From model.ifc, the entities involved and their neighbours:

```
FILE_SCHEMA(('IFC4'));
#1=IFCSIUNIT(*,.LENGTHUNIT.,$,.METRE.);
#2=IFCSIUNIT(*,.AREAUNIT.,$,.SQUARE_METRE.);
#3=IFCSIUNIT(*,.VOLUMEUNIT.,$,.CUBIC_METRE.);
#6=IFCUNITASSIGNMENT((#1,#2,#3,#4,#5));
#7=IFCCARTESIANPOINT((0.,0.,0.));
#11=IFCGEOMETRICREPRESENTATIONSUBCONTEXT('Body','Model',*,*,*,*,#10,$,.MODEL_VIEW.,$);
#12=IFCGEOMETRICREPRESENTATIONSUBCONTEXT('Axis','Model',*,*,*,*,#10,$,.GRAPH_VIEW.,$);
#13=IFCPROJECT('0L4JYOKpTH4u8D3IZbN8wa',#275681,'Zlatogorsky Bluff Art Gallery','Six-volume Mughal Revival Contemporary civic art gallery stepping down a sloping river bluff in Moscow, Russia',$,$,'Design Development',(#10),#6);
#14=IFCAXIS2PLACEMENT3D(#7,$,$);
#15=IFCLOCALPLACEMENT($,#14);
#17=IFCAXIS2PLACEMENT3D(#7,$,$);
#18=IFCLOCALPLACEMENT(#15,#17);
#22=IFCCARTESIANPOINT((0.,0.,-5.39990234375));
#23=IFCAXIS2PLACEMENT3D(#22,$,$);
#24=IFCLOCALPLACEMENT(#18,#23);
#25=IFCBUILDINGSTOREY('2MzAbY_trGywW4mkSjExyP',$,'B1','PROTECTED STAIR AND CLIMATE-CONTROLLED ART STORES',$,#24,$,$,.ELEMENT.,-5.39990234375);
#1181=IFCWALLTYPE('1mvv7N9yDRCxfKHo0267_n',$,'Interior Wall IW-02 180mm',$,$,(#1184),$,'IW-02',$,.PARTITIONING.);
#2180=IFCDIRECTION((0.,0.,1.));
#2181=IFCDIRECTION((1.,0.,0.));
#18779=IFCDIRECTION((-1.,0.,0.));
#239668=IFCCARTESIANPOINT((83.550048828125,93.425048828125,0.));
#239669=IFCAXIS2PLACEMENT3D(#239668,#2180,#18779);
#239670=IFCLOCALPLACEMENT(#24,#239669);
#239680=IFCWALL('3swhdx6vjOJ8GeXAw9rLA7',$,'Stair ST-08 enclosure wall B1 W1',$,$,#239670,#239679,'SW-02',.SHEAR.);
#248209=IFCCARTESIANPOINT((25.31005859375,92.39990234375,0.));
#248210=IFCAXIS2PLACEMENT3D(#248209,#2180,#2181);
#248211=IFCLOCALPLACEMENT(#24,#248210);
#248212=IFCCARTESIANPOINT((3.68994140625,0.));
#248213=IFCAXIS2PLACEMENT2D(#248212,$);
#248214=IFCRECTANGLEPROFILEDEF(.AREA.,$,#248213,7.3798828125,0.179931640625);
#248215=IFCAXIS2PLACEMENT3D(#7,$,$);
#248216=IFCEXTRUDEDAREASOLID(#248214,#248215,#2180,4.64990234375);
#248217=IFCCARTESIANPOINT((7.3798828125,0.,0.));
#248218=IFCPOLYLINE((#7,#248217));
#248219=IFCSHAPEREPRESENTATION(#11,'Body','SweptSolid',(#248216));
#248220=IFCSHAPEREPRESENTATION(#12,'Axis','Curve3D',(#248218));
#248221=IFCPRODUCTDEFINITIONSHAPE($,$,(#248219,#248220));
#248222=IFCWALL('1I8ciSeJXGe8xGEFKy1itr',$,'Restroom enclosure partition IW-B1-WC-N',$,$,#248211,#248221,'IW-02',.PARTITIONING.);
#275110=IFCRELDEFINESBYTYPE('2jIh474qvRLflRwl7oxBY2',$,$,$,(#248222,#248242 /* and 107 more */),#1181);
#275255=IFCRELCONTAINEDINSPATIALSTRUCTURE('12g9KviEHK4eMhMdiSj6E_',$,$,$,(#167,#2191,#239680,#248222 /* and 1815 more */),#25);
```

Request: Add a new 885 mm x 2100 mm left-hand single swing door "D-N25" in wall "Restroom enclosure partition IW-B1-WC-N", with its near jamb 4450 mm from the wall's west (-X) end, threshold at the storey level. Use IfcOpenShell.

```python
import numpy as np
import ifcopenshell
import ifcopenshell.api.feature
import ifcopenshell.api.geometry
import ifcopenshell.api.root
import ifcopenshell.api.spatial
import ifcopenshell.geom
import ifcopenshell.util.element
import ifcopenshell.util.placement
import ifcopenshell.util.representation
import ifcopenshell.util.shape
import ifcopenshell.util.unit

model = ifcopenshell.open("model.ifc")
unit_scale = ifcopenshell.util.unit.calculate_unit_scale(model)
settings = ifcopenshell.geom.settings()


def volume(element):
    """Net volume in cubic metres, openings subtracted."""
    shape = ifcopenshell.geom.create_shape(settings, element)
    return ifcopenshell.util.shape.get_volume(shape.geometry)


wall = model.by_guid("1I8ciSeJXGe8xGEFKy1itr")
storey = ifcopenshell.util.element.get_container(wall, ifc_class="IfcBuildingStorey")
context = ifcopenshell.util.representation.get_context(model, "Model", "Body", "MODEL_VIEW")
before = volume(wall)

width, height, from_end, sill = 0.885, 2.1, 4.45, 0.0  # metres

# The wall runs along its own X axis, and the end named is its -X end.
wall_shape = ifcopenshell.geom.create_shape(settings, wall)
x, y, z = ifcopenshell.util.shape.get_vertices(wall_shape.geometry).T
start = x.min() + from_end
face, thickness = float(y.min()), float(y.max() - y.min())
wall_matrix = ifcopenshell.util.placement.get_local_placement(wall.ObjectPlacement)
level = ifcopenshell.util.placement.get_local_placement(storey.ObjectPlacement)[2, 3]


def in_wall(x, y):
    """Placement at x, y metres in the wall's axes, at sill height."""
    matrix = wall_matrix.copy()
    matrix[:, 3] = wall_matrix @ np.array([x / unit_scale, y / unit_scale, 0.0, 1.0])
    matrix[2, 3] = level + sill / unit_scale
    return matrix


# Opening: a box that overshoots both wall faces by 50 mm.
opening = ifcopenshell.api.root.create_entity(model, ifc_class="IfcOpeningElement", predefined_type="OPENING")
box = ifcopenshell.api.geometry.add_wall_representation(
    model, context=context, length=width, height=height, thickness=thickness + 0.1
)
ifcopenshell.api.geometry.assign_representation(model, product=opening, representation=box)
ifcopenshell.api.geometry.edit_object_placement(model, product=opening, matrix=in_wall(start, face - 0.05), is_si=False)
ifcopenshell.api.feature.add_feature(model, feature=opening, element=wall)

door = ifcopenshell.api.root.create_entity(model, ifc_class="IfcDoor", name="D-N25", predefined_type="DOOR")
door.OverallWidth, door.OverallHeight = width / unit_scale, height / unit_scale
door.OperationType = "SINGLE_SWING_LEFT"
body = ifcopenshell.api.geometry.add_door_representation(
    model,
    context=context,
    overall_width=door.OverallWidth,
    overall_height=door.OverallHeight,
    operation_type="SINGLE_SWING_LEFT",
    lining_properties={"LiningDepth": thickness / unit_scale, "ThresholdDepth": thickness / unit_scale},
)
ifcopenshell.api.geometry.assign_representation(model, product=door, representation=body)
ifcopenshell.api.spatial.assign_container(model, products=[door], relating_structure=storey)
ifcopenshell.api.feature.add_filling(model, opening=opening, element=door)

# The lining spans the wall, so the door starts at the wall face.
ifcopenshell.api.geometry.edit_object_placement(model, product=door, matrix=in_wall(start, face), is_si=False)

after = volume(wall)

print(f"wall volume {before:.3f} -> {after:.3f} m3")

model.write("model_rev.ifc")
```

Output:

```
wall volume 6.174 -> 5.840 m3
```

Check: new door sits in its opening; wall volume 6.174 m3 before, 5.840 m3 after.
